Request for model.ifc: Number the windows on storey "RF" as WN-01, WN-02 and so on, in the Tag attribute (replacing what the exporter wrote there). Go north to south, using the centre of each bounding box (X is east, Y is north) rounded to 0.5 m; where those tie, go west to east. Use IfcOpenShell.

First a look at what the model holds.

```python
import ifcopenshell
import ifcopenshell.util.element
import ifcopenshell.util.placement

model = ifcopenshell.open("model.ifc")
print(model.schema)
storey = next(s for s in model.by_type("IfcBuildingStorey") if s.Name == "RF")
windows = [e for e in ifcopenshell.util.element.get_decomposition(storey) if e.is_a("IfcWindow")]
for e in sorted(windows, key=lambda e: e.id()):
    origin = ifcopenshell.util.placement.get_local_placement(e.ObjectPlacement)[:3, 3]
    print(e.id(), e.Tag, e.Name, origin.round(2) + 0.0, sep=" | ")
```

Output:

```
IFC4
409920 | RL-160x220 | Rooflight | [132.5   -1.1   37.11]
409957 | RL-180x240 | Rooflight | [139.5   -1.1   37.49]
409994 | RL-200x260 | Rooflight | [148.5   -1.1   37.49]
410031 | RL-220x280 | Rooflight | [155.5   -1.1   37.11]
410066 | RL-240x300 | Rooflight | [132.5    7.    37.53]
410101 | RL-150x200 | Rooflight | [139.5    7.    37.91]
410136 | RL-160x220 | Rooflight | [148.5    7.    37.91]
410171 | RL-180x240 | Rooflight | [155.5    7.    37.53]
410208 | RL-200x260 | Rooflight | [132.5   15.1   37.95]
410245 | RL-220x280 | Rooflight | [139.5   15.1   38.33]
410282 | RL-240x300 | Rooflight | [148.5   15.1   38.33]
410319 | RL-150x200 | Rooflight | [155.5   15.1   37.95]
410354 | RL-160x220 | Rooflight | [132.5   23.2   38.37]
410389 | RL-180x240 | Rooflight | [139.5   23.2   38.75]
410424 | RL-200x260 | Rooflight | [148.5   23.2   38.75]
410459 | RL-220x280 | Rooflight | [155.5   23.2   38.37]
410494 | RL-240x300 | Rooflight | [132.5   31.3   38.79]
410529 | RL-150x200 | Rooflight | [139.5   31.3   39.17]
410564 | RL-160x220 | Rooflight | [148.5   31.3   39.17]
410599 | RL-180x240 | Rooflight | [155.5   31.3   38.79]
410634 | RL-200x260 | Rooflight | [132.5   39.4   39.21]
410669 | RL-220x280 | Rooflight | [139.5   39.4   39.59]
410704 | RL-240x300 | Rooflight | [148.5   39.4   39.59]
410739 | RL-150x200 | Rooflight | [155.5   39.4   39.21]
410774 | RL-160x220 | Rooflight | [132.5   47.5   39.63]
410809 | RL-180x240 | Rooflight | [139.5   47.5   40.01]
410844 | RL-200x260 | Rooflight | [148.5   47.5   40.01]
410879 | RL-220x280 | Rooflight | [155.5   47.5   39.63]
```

```python
import ifcopenshell
import ifcopenshell.geom
import ifcopenshell.util.element
import ifcopenshell.util.shape

model = ifcopenshell.open("model.ifc")
settings = ifcopenshell.geom.settings()
settings.set("use-world-coords", True)


def centre(element):
    shape = ifcopenshell.geom.create_shape(settings, element)
    return ifcopenshell.util.shape.get_bbox_centroid(shape.geometry)


storey = next(s for s in model.by_type("IfcBuildingStorey") if s.Name == "RF")
windows = [e for e in ifcopenshell.util.element.get_decomposition(storey) if e.is_a("IfcWindow")]

# Insertion points can sit at a corner or the storey origin, so sort by the geometry (in metres).
centres = {e: centre(e) for e in windows}
windows.sort(key=lambda e: (-round(centres[e][1] / 0.5), centres[e][0]))

for i, e in enumerate(windows, start=1):
    number = f"WN-{i:02d}"
    e.Tag = number
    print(e.id(), number)

model.write("model_edited.ifc")
```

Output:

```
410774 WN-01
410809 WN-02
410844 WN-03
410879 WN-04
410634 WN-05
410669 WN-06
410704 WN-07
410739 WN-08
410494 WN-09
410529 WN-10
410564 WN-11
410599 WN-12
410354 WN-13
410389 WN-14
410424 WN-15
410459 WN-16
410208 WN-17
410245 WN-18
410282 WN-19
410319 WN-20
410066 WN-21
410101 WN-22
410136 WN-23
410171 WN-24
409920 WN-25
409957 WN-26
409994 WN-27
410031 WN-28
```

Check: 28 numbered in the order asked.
